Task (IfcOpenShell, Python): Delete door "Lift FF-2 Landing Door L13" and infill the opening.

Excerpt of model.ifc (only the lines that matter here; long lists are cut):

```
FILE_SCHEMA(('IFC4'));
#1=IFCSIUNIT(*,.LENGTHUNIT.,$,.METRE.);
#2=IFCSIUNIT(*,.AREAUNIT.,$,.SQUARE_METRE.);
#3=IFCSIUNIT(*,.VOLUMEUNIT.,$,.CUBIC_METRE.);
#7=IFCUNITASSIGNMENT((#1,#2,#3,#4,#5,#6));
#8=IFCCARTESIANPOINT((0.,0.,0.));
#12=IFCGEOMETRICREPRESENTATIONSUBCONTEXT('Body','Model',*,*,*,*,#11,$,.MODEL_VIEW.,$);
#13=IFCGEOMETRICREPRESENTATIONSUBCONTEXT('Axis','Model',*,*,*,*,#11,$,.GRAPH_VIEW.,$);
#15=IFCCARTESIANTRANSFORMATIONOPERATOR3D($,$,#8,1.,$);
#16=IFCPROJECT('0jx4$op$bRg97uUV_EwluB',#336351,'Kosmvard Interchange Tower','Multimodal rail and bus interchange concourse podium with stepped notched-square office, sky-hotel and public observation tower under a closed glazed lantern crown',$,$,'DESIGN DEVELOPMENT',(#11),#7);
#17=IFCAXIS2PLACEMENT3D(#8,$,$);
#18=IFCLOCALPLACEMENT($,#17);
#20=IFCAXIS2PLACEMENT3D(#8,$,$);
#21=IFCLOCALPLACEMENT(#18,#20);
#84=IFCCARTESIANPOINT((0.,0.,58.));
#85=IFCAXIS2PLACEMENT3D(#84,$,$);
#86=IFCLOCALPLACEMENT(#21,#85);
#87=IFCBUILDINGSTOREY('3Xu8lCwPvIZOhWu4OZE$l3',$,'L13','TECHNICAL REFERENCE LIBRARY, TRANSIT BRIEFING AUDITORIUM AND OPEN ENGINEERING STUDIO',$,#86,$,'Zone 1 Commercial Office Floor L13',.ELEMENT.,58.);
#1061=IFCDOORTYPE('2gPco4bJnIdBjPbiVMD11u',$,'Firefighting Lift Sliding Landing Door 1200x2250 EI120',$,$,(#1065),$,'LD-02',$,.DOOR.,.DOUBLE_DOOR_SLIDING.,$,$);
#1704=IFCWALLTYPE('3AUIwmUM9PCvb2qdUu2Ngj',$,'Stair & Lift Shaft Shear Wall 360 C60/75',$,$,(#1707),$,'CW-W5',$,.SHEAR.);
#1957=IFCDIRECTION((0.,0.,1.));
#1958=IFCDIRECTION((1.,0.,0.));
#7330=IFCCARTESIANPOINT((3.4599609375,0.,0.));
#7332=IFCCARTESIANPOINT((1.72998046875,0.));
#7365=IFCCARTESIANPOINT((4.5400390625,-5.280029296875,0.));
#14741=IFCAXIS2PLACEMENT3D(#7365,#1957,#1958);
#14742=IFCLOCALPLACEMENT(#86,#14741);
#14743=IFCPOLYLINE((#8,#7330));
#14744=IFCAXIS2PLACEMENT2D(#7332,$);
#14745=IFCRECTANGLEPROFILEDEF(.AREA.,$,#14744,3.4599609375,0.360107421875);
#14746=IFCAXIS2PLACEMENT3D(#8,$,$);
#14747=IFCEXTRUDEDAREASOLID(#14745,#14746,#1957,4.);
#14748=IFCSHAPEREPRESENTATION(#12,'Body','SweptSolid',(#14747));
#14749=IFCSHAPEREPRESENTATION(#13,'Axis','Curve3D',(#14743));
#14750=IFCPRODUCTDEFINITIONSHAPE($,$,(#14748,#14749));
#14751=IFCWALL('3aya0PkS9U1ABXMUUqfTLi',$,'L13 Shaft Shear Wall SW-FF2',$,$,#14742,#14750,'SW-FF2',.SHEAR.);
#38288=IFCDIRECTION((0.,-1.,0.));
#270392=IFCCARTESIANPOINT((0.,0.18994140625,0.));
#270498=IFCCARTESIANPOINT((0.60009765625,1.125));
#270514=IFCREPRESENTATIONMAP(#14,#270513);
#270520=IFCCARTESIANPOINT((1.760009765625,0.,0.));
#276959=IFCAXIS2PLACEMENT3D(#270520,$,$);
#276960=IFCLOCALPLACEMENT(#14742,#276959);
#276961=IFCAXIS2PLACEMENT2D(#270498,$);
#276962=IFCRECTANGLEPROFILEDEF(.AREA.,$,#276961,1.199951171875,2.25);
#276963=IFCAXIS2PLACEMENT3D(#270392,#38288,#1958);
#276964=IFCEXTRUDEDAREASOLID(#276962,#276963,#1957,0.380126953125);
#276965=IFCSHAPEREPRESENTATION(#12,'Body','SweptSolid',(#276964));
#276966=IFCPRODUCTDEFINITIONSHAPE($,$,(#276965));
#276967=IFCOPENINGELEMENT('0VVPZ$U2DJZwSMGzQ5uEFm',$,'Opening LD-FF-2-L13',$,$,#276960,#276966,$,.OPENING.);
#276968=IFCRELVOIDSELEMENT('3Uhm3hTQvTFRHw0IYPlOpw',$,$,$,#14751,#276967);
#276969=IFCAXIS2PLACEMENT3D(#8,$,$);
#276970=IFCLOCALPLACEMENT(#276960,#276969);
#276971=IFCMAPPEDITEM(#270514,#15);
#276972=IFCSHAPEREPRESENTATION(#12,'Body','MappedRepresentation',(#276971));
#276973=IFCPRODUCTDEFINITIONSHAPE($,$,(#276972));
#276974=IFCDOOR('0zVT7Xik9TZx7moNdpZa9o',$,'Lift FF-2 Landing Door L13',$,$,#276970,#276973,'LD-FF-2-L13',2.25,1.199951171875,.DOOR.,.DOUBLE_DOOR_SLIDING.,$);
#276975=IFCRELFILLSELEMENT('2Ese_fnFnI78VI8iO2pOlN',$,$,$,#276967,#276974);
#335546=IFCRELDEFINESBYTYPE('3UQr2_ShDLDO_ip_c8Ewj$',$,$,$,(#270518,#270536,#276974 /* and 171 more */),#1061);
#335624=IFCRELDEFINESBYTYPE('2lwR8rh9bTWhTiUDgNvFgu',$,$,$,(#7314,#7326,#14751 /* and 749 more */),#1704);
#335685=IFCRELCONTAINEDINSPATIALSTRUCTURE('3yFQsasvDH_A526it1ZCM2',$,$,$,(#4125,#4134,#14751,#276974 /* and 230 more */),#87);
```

```python
import ifcopenshell
import ifcopenshell.api.feature
import ifcopenshell.api.root
import ifcopenshell.geom
import ifcopenshell.util.shape

model = ifcopenshell.open("model.ifc")
settings = ifcopenshell.geom.settings()


def volume(element):
    """Net volume in cubic metres, openings subtracted."""
    shape = ifcopenshell.geom.create_shape(settings, element)
    return ifcopenshell.util.shape.get_volume(shape.geometry)


door = model.by_guid("0zVT7Xik9TZx7moNdpZa9o")
opening = door.FillsVoids[0].RelatingOpeningElement
wall = opening.VoidsElements[0].RelatingBuildingElement
before = volume(wall)

ifcopenshell.api.root.remove_product(model, product=door)
ifcopenshell.api.feature.remove_feature(model, feature=opening)

after = volume(wall)

print(f"wall volume {before:.3f} -> {after:.3f} m3")

model.write("model_v2.ifc")
```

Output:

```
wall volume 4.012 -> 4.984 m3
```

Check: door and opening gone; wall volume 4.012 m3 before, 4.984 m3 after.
